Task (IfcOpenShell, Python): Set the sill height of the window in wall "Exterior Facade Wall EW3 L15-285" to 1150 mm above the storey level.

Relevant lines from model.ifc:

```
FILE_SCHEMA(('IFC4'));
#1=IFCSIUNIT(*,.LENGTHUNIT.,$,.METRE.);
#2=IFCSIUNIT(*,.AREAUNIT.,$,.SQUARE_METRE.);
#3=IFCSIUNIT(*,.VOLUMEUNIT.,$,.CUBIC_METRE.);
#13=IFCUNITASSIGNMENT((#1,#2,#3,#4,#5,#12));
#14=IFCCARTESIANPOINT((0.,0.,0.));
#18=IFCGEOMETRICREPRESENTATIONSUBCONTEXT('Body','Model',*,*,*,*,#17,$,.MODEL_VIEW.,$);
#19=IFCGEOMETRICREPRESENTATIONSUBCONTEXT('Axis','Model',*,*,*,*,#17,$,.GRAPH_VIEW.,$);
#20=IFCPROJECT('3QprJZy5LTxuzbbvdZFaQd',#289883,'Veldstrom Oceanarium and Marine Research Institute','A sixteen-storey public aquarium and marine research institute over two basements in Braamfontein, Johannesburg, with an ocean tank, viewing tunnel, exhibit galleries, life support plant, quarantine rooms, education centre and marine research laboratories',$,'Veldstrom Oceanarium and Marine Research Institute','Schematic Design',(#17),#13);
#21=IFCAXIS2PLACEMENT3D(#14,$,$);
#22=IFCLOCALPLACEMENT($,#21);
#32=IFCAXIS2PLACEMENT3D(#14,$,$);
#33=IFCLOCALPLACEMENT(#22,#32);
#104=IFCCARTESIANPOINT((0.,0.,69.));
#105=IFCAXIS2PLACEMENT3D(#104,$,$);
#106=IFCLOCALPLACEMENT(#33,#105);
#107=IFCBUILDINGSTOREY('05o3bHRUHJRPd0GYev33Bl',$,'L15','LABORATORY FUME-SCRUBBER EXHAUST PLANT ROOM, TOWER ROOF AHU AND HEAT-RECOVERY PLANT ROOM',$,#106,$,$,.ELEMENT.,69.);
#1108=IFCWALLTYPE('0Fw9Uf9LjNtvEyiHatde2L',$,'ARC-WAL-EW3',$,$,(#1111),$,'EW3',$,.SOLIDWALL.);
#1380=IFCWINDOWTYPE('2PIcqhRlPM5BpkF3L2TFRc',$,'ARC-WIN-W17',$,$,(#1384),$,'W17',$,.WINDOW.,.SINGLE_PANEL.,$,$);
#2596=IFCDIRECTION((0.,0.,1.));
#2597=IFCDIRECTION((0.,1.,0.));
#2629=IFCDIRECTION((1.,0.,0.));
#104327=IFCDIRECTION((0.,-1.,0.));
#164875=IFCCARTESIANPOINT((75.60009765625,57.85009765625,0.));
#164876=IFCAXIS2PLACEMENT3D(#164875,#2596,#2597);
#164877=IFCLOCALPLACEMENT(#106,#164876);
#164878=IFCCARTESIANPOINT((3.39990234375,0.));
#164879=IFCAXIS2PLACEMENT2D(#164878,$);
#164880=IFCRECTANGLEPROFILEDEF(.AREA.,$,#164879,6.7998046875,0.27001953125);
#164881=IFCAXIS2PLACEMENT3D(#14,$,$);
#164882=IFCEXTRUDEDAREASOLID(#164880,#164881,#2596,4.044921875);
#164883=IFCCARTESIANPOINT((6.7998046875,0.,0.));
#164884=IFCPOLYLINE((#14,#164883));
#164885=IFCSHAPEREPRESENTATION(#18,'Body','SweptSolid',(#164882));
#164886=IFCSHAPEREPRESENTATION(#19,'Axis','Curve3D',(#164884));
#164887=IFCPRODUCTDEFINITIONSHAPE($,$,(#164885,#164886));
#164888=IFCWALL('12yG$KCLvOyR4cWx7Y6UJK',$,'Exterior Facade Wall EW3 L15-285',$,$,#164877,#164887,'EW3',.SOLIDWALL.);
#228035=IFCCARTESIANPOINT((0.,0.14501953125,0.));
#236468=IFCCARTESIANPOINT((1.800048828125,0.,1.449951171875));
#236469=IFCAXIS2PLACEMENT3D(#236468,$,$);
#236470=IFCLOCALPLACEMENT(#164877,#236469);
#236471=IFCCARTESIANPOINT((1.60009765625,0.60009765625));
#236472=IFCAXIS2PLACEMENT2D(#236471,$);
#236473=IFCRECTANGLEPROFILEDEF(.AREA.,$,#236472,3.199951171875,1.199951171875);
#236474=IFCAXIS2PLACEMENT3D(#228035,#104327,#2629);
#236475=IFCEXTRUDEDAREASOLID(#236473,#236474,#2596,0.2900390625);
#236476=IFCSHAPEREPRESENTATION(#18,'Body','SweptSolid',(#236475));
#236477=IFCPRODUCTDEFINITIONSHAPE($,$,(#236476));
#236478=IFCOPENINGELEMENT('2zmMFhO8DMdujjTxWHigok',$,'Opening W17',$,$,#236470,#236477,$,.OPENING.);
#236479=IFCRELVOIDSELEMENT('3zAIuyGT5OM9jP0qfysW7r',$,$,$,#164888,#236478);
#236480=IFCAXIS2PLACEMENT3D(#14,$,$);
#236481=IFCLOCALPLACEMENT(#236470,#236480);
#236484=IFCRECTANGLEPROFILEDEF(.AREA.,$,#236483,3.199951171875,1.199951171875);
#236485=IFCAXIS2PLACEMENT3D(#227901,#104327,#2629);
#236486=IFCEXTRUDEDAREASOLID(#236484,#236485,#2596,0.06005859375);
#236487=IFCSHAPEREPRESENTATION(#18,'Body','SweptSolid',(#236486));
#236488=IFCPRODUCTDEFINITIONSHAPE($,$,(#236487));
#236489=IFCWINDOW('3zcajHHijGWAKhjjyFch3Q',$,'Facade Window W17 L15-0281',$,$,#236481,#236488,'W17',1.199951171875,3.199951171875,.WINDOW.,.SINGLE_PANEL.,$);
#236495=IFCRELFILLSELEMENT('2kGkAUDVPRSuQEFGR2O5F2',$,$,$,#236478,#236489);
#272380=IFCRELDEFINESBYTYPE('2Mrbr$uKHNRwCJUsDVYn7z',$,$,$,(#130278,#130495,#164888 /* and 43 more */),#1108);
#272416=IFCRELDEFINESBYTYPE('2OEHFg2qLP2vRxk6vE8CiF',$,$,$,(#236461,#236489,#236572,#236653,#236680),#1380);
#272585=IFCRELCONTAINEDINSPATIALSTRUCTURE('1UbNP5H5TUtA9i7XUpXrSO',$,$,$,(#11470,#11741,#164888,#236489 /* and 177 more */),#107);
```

```python
import numpy as np
import ifcopenshell
import ifcopenshell.api.geometry
import ifcopenshell.geom
import ifcopenshell.util.element
import ifcopenshell.util.placement
import ifcopenshell.util.shape
import ifcopenshell.util.unit

model = ifcopenshell.open("model.ifc")
unit_scale = ifcopenshell.util.unit.calculate_unit_scale(model)

window = model.by_guid("3zcajHHijGWAKhjjyFch3Q")
opening = window.FillsVoids[0].RelatingOpeningElement
storey = ifcopenshell.util.element.get_container(window, ifc_class="IfcBuildingStorey")
level = ifcopenshell.util.placement.get_local_placement(storey.ObjectPlacement)[2, 3]

# The opening's origin need not be at the sill, so measure its lowest point.
shape = ifcopenshell.geom.create_shape(ifcopenshell.geom.settings(), opening)
bottom = ifcopenshell.util.shape.get_shape_bottom_elevation(shape, shape.geometry) / unit_scale
dz = level + 1.15 - bottom

shift = np.array([0.0, 0.0, dz])
# The window is placed relative to its opening, so it follows when the opening moves.
matrix = ifcopenshell.util.placement.get_local_placement(opening.ObjectPlacement)
matrix[:3, 3] += shift
ifcopenshell.api.geometry.edit_object_placement(
    model, product=opening, matrix=matrix, is_si=False, should_transform_children=True
)

print(f"moved by {dz * unit_scale:+.3f} m")

model.write("model-out.ifc")
```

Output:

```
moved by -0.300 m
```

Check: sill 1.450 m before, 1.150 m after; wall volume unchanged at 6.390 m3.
